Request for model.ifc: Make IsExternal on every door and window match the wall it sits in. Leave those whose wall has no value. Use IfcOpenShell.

First a look at what the model holds.

```python
import ifcopenshell
import ifcopenshell.util.element

model = ifcopenshell.open("model.ifc")
print(model.schema)
seen = {}
for e in model.by_type("IfcDoor") + model.by_type("IfcWindow"):
    if not e.FillsVoids:
        continue
    host = e.FillsVoids[0].RelatingOpeningElement.VoidsElements[0].RelatingBuildingElement
    own = ifcopenshell.util.element.get_pset(e, f"Pset_{e.is_a()[3:].removesuffix('StandardCase')}Common", "IsExternal")
    wall = ifcopenshell.util.element.get_pset(host, "Pset_WallCommon", "IsExternal")
    seen[e.is_a(), own, wall] = seen.get((e.is_a(), own, wall), 0) + 1
for (cls, own, wall), count in sorted(seen.items(), key=str):
    print(count, cls, "IsExternal:", own, "| host wall:", wall)
```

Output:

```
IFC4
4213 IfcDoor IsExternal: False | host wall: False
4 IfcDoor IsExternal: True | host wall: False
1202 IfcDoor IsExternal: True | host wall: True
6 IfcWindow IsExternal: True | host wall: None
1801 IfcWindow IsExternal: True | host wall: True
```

```python
import ifcopenshell
import ifcopenshell.api.pset
import ifcopenshell.util.element

model = ifcopenshell.open("model.ifc")

count = 0
for ifc_class, pset_name in (("IfcDoor", "Pset_DoorCommon"), ("IfcWindow", "Pset_WindowCommon")):
    for e in model.by_type(ifc_class):
        if not e.FillsVoids:
            continue
        host = e.FillsVoids[0].RelatingOpeningElement.VoidsElements[0].RelatingBuildingElement
        external = ifcopenshell.util.element.get_pset(host, "Pset_WallCommon", "IsExternal")
        if external is None or ifcopenshell.util.element.get_pset(e, pset_name, "IsExternal") == external:
            continue
        pset = ifcopenshell.api.pset.add_pset(model, product=e, name=pset_name)
        ifcopenshell.api.pset.edit_pset(model, pset=pset, properties={"IsExternal": external})
        count += 1

print(count, "updated")

model.write("model-out.ifc")
```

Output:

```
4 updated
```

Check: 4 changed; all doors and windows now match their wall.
